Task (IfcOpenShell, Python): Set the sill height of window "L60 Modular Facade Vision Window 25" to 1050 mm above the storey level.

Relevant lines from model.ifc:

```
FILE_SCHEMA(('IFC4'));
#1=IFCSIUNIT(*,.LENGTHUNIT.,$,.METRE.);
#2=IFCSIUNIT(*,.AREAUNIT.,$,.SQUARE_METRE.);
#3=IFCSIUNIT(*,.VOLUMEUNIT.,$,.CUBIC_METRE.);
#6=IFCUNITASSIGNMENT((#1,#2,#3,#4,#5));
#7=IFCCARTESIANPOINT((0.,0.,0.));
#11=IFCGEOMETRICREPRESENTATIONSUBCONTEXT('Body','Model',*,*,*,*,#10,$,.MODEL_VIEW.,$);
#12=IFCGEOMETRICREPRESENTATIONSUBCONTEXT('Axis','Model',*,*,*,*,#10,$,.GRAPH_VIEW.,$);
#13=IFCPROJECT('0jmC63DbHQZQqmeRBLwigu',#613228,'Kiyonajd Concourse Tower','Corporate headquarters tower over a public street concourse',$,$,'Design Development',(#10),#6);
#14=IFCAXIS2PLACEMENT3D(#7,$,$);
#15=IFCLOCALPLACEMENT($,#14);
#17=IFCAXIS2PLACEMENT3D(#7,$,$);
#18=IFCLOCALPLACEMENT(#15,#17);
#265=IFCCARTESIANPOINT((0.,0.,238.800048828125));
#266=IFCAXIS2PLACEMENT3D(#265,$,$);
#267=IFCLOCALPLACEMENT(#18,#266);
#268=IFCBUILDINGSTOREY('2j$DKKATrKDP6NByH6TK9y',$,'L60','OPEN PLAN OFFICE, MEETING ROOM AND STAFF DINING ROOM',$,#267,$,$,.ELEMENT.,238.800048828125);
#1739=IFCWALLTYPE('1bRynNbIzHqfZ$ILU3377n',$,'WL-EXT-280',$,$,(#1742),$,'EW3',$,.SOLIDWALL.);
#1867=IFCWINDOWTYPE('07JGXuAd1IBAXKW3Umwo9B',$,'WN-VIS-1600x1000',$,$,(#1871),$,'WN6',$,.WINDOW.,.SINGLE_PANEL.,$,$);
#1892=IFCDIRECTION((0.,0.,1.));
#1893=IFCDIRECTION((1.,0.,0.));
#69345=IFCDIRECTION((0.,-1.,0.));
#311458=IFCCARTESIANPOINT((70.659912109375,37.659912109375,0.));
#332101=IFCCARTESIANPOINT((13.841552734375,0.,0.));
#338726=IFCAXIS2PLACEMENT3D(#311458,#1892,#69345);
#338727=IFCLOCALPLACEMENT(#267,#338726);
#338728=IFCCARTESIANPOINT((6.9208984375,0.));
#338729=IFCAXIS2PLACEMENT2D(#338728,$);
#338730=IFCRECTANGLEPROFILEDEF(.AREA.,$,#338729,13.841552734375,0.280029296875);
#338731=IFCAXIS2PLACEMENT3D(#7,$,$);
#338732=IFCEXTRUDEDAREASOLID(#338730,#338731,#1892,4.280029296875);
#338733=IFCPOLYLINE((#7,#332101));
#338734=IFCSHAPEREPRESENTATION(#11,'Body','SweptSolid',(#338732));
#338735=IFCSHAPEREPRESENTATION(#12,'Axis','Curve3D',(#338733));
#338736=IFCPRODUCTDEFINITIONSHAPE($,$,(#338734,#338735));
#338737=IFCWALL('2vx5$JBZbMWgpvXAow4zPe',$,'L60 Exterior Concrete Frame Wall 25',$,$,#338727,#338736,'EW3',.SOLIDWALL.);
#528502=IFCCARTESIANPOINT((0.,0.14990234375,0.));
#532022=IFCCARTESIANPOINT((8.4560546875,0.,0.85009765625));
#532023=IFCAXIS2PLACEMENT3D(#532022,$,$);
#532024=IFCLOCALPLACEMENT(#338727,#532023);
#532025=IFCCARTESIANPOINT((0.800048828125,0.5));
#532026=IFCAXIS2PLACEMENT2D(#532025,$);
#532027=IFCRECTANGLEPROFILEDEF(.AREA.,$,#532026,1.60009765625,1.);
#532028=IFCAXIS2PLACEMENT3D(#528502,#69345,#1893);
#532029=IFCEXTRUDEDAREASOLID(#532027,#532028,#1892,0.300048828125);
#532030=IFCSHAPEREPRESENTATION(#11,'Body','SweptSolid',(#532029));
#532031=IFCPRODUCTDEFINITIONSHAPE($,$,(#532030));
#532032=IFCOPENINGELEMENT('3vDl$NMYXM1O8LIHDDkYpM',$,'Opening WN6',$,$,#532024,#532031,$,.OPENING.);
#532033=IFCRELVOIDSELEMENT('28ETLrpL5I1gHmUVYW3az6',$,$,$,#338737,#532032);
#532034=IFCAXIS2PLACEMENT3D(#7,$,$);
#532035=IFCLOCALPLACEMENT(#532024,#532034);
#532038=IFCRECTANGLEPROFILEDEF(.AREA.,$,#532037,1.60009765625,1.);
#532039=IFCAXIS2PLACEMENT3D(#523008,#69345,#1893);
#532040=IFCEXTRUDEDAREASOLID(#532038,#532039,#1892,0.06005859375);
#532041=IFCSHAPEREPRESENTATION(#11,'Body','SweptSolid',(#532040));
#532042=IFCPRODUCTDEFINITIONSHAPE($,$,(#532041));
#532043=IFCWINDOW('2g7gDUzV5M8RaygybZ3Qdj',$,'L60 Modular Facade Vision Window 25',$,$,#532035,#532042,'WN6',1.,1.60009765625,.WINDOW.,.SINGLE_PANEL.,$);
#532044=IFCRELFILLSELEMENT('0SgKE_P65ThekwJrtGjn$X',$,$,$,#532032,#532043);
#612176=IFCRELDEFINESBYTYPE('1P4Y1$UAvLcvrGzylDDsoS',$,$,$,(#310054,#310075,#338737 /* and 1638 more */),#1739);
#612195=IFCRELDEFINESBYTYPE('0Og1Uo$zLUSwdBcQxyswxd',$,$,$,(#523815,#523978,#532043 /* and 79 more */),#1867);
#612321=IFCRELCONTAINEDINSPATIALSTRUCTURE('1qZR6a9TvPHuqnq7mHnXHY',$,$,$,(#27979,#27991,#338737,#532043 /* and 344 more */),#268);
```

```python
import numpy as np
import ifcopenshell
import ifcopenshell.api.geometry
import ifcopenshell.geom
import ifcopenshell.util.element
import ifcopenshell.util.placement
import ifcopenshell.util.shape
import ifcopenshell.util.unit

model = ifcopenshell.open("model.ifc")
unit_scale = ifcopenshell.util.unit.calculate_unit_scale(model)

window = model.by_guid("2g7gDUzV5M8RaygybZ3Qdj")
opening = window.FillsVoids[0].RelatingOpeningElement
storey = ifcopenshell.util.element.get_container(window, ifc_class="IfcBuildingStorey")
level = ifcopenshell.util.placement.get_local_placement(storey.ObjectPlacement)[2, 3]

# The opening's origin need not be at the sill, so measure its lowest point.
shape = ifcopenshell.geom.create_shape(ifcopenshell.geom.settings(), opening)
bottom = ifcopenshell.util.shape.get_shape_bottom_elevation(shape, shape.geometry) / unit_scale
dz = level + 1.05 / unit_scale - bottom

shift = np.array([0.0, 0.0, dz])
# The window is placed relative to its opening, so it follows when the opening moves.
matrix = ifcopenshell.util.placement.get_local_placement(opening.ObjectPlacement)
matrix[:3, 3] += shift
ifcopenshell.api.geometry.edit_object_placement(
    model, product=opening, matrix=matrix, is_si=False, should_transform_children=True
)

print(f"moved by {dz * unit_scale:+.3f} m")

model.write("model_rev.ifc")
```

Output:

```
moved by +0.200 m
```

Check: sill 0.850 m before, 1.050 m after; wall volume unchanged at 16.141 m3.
